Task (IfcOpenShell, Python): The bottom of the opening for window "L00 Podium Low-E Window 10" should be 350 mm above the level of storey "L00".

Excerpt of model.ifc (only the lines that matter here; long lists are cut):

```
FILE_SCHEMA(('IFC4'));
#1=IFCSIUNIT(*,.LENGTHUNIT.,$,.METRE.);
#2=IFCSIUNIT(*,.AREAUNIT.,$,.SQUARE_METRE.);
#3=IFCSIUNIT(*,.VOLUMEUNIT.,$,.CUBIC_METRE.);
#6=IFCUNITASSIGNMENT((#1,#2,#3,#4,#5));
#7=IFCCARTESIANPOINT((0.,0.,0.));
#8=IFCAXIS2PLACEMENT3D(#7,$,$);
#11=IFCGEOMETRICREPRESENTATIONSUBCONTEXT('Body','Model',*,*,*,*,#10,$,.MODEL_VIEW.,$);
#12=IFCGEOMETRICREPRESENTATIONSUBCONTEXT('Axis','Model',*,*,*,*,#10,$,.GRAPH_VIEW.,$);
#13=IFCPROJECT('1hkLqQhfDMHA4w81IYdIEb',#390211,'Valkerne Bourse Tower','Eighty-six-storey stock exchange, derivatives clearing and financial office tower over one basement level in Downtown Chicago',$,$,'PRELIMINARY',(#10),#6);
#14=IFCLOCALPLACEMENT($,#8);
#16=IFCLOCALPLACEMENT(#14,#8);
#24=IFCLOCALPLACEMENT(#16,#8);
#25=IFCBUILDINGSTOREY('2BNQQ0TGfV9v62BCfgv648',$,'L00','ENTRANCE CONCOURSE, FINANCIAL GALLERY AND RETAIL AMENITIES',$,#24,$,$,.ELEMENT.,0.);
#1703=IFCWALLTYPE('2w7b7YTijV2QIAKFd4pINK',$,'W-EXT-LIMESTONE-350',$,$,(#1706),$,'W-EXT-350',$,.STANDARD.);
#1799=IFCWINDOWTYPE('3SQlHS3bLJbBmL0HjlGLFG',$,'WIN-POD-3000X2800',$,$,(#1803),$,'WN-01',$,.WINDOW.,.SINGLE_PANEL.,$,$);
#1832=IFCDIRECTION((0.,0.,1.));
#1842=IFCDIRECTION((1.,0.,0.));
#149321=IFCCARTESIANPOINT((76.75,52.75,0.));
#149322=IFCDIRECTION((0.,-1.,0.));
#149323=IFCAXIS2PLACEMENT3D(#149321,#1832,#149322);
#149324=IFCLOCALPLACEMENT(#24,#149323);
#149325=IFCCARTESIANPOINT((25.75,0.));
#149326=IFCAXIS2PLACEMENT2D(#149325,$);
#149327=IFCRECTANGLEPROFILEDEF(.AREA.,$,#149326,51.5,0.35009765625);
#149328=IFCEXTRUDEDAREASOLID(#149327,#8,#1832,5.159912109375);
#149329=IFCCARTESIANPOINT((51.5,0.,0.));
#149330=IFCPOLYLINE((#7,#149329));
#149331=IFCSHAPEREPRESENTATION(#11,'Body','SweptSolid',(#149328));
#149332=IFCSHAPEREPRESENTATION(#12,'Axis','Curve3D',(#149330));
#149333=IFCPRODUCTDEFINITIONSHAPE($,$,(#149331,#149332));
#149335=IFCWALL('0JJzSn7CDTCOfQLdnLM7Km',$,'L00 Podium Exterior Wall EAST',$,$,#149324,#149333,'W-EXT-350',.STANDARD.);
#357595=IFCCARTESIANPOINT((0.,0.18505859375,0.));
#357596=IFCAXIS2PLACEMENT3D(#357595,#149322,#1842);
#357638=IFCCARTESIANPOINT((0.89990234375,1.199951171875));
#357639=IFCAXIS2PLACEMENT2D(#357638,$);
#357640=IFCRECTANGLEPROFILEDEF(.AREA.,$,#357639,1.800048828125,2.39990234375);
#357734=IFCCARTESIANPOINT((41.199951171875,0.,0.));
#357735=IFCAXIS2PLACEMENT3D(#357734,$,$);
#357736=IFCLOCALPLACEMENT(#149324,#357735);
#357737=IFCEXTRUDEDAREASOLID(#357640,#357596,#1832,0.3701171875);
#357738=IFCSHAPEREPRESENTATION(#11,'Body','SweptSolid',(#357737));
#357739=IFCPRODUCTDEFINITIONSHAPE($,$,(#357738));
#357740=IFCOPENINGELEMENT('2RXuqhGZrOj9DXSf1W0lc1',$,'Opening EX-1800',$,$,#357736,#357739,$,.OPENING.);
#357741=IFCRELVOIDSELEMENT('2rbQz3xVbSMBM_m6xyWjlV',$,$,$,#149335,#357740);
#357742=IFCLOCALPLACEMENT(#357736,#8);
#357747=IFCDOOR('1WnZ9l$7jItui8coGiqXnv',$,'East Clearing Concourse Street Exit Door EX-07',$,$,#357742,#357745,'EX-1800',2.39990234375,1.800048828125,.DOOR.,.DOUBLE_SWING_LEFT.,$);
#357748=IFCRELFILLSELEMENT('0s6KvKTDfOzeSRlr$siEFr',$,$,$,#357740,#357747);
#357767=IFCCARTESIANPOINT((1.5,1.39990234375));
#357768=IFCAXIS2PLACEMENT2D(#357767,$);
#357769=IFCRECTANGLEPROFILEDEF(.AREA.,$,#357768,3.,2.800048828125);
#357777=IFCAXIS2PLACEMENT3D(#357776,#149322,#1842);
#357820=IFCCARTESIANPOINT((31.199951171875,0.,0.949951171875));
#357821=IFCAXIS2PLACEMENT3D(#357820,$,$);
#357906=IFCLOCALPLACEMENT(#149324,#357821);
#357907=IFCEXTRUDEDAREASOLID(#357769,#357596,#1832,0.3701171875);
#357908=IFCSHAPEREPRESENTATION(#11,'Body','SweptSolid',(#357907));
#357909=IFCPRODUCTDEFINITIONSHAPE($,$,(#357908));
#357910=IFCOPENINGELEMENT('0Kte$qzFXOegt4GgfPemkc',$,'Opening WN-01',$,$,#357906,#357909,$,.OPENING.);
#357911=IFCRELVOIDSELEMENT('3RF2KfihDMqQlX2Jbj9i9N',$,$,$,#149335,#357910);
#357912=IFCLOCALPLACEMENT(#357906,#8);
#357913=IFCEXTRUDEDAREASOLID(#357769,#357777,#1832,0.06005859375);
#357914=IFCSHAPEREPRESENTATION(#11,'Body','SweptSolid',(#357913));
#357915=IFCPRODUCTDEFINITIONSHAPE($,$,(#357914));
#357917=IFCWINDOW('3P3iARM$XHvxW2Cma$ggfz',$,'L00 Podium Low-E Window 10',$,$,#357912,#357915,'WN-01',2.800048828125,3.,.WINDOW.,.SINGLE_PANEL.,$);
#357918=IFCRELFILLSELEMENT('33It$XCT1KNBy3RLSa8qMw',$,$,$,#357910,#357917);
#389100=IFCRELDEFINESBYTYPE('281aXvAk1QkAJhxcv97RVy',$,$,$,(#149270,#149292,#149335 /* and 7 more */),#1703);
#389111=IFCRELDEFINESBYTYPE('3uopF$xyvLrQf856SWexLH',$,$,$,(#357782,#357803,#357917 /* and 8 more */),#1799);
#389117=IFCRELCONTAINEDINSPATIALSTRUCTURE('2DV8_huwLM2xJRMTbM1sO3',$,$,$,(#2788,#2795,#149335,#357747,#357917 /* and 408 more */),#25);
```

```python
import numpy as np
import ifcopenshell
import ifcopenshell.api.geometry
import ifcopenshell.geom
import ifcopenshell.util.element
import ifcopenshell.util.placement
import ifcopenshell.util.shape
import ifcopenshell.util.unit

model = ifcopenshell.open("model.ifc")
unit_scale = ifcopenshell.util.unit.calculate_unit_scale(model)

window = model.by_guid("3P3iARM$XHvxW2Cma$ggfz")
opening = window.FillsVoids[0].RelatingOpeningElement
storey = ifcopenshell.util.element.get_container(window, ifc_class="IfcBuildingStorey")
level = ifcopenshell.util.placement.get_local_placement(storey.ObjectPlacement)[2, 3]

# The opening's origin need not be at the sill, so measure its lowest point.
shape = ifcopenshell.geom.create_shape(ifcopenshell.geom.settings(), opening)
bottom = ifcopenshell.util.shape.get_shape_bottom_elevation(shape, shape.geometry) / unit_scale
dz = level + 0.35 / unit_scale - bottom

shift = np.array([0.0, 0.0, dz])
# The window is placed relative to its opening, so it follows when the opening moves.
matrix = ifcopenshell.util.placement.get_local_placement(opening.ObjectPlacement)
matrix[:3, 3] += shift
ifcopenshell.api.geometry.edit_object_placement(
    model, product=opening, matrix=matrix, is_si=False, should_transform_children=True
)

print(f"moved by {dz * unit_scale:+.3f} m")

model.write("model_updated.ifc")
```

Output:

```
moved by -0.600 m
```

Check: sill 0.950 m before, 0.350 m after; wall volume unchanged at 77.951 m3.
